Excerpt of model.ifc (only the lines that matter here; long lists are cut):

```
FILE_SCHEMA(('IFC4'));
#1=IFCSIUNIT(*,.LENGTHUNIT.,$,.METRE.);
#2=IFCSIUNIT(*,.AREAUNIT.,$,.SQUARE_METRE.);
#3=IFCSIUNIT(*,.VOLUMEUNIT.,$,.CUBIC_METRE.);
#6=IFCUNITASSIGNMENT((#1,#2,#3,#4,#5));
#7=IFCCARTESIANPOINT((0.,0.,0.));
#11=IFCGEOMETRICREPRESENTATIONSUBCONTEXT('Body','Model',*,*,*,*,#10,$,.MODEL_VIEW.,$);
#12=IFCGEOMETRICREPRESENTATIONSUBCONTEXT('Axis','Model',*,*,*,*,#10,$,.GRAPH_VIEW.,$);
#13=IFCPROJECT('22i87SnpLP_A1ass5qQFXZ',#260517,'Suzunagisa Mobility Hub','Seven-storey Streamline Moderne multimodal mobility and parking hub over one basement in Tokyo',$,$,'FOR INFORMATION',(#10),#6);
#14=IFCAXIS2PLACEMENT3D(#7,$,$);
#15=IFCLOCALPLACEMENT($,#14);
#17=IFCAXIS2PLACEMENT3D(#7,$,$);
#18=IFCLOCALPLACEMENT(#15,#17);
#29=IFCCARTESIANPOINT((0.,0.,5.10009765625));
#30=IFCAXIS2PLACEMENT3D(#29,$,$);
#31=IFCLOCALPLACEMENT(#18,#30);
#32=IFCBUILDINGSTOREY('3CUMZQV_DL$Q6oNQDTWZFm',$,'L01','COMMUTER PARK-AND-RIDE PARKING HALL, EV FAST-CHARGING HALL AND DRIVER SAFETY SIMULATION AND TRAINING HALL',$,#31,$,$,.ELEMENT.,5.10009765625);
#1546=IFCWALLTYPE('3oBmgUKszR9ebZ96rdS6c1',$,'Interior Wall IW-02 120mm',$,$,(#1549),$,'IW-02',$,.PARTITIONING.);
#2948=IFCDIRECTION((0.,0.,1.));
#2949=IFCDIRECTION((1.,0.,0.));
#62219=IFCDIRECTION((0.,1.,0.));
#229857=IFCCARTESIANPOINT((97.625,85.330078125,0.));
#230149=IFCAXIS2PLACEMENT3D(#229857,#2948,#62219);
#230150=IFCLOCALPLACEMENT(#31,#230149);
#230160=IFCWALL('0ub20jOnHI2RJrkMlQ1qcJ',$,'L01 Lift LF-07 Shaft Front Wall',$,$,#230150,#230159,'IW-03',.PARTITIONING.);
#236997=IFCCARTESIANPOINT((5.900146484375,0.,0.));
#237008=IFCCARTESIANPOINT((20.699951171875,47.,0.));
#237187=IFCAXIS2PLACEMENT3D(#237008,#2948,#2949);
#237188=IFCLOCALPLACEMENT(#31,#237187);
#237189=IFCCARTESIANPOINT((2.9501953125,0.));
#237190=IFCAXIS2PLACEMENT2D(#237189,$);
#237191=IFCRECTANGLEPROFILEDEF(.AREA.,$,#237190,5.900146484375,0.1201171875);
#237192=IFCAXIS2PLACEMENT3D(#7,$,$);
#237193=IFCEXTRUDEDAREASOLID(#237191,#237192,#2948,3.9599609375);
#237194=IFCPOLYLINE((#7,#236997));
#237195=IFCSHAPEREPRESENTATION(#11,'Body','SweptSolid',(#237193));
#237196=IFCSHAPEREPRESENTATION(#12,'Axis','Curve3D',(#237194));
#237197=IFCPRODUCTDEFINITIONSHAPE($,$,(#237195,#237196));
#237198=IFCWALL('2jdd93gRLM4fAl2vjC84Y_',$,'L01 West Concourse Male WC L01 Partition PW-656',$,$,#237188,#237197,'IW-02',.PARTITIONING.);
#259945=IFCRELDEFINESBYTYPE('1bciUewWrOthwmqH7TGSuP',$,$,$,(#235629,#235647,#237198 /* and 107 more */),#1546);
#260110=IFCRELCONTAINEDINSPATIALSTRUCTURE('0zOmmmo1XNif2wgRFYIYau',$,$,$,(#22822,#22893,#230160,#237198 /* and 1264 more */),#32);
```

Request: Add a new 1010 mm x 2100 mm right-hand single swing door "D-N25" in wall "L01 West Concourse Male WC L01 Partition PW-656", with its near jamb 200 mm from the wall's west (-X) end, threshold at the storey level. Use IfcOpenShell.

```python
import numpy as np
import ifcopenshell
import ifcopenshell.api.feature
import ifcopenshell.api.geometry
import ifcopenshell.api.root
import ifcopenshell.api.spatial
import ifcopenshell.geom
import ifcopenshell.util.element
import ifcopenshell.util.placement
import ifcopenshell.util.representation
import ifcopenshell.util.shape
import ifcopenshell.util.unit

model = ifcopenshell.open("model.ifc")
unit_scale = ifcopenshell.util.unit.calculate_unit_scale(model)
settings = ifcopenshell.geom.settings()


def volume(element):
    """Net volume in cubic metres, openings subtracted."""
    shape = ifcopenshell.geom.create_shape(settings, element)
    return ifcopenshell.util.shape.get_volume(shape.geometry)


wall = model.by_guid("2jdd93gRLM4fAl2vjC84Y_")
storey = ifcopenshell.util.element.get_container(wall, ifc_class="IfcBuildingStorey")
context = ifcopenshell.util.representation.get_context(model, "Model", "Body", "MODEL_VIEW")
before = volume(wall)

width, height, from_end, sill = 1.01, 2.1, 0.2, 0.0  # metres

# The wall runs along its own X axis, and the end named is its -X end.
wall_shape = ifcopenshell.geom.create_shape(settings, wall)
x, y, z = ifcopenshell.util.shape.get_vertices(wall_shape.geometry).T
start = x.min() + from_end
face, thickness = float(y.min()), float(y.max() - y.min())
wall_matrix = ifcopenshell.util.placement.get_local_placement(wall.ObjectPlacement)
level = ifcopenshell.util.placement.get_local_placement(storey.ObjectPlacement)[2, 3]


def in_wall(x, y):
    """Placement at x, y metres in the wall's axes, at sill height."""
    matrix = wall_matrix.copy()
    matrix[:, 3] = wall_matrix @ np.array([x / unit_scale, y / unit_scale, 0.0, 1.0])
    matrix[2, 3] = level + sill / unit_scale
    return matrix


# Opening: a box that overshoots both wall faces by 50 mm.
opening = ifcopenshell.api.root.create_entity(model, ifc_class="IfcOpeningElement", predefined_type="OPENING")
box = ifcopenshell.api.geometry.add_wall_representation(
    model, context=context, length=width, height=height, thickness=thickness + 0.1
)
ifcopenshell.api.geometry.assign_representation(model, product=opening, representation=box)
ifcopenshell.api.geometry.edit_object_placement(model, product=opening, matrix=in_wall(start, face - 0.05), is_si=False)
ifcopenshell.api.feature.add_feature(model, feature=opening, element=wall)

door = ifcopenshell.api.root.create_entity(model, ifc_class="IfcDoor", name="D-N25", predefined_type="DOOR")
door.OverallWidth, door.OverallHeight = width / unit_scale, height / unit_scale
door.OperationType = "SINGLE_SWING_RIGHT"
body = ifcopenshell.api.geometry.add_door_representation(
    model,
    context=context,
    overall_width=door.OverallWidth,
    overall_height=door.OverallHeight,
    operation_type="SINGLE_SWING_RIGHT",
    lining_properties={"LiningDepth": thickness / unit_scale, "ThresholdDepth": thickness / unit_scale},
)
ifcopenshell.api.geometry.assign_representation(model, product=door, representation=body)
ifcopenshell.api.spatial.assign_container(model, products=[door], relating_structure=storey)
ifcopenshell.api.feature.add_filling(model, opening=opening, element=door)

# The lining spans the wall, so the door starts at the wall face.
ifcopenshell.api.geometry.edit_object_placement(model, product=door, matrix=in_wall(start, face), is_si=False)

after = volume(wall)

print(f"wall volume {before:.3f} -> {after:.3f} m3")

model.write("model-out.ifc")
```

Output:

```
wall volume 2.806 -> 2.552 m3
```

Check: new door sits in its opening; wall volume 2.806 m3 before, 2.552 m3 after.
